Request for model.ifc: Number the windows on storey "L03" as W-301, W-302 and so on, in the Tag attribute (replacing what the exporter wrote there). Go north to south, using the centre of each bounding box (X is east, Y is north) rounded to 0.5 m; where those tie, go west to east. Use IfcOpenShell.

First a look at what the model holds.

```python
import ifcopenshell
import ifcopenshell.util.element
import ifcopenshell.util.placement

model = ifcopenshell.open("model.ifc")
print(model.schema)
storey = next(s for s in model.by_type("IfcBuildingStorey") if s.Name == "L03")
windows = [e for e in ifcopenshell.util.element.get_decomposition(storey) if e.is_a("IfcWindow")]
for e in sorted(windows, key=lambda e: e.id()):
    origin = ifcopenshell.util.placement.get_local_placement(e.ObjectPlacement)[:3, 3]
    print(e.id(), e.Tag, e.Name, origin.round(2) + 0.0, sep=" | ")
```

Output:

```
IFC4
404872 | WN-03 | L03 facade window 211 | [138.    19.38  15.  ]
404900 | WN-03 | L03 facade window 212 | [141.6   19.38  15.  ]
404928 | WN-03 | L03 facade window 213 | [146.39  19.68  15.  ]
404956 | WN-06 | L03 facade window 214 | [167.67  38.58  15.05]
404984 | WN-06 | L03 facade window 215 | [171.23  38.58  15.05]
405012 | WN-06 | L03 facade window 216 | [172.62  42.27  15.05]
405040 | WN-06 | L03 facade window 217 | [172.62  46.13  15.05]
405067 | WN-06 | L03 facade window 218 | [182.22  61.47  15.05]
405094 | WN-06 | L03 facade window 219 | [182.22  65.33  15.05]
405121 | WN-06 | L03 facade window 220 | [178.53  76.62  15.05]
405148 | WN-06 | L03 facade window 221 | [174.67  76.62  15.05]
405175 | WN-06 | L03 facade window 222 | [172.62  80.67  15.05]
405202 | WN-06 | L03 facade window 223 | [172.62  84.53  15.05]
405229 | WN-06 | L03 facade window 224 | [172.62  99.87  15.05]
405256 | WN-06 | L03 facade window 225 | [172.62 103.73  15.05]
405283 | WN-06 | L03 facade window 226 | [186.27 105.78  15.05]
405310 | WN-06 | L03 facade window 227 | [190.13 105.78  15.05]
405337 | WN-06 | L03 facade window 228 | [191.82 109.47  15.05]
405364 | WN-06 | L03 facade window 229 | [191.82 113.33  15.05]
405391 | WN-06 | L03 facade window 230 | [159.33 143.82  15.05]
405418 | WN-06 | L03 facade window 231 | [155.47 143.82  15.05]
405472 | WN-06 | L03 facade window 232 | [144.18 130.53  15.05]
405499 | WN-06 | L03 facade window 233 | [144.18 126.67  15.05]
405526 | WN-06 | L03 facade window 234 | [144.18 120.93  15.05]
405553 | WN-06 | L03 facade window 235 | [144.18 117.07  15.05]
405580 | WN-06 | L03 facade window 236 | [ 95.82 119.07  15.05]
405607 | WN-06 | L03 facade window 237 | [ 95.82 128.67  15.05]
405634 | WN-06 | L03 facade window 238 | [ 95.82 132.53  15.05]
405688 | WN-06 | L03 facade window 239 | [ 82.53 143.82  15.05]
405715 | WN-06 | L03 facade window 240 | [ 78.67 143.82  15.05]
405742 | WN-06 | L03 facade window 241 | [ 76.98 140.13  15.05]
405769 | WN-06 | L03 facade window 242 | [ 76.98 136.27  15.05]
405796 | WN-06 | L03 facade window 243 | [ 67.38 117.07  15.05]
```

```python
import ifcopenshell
import ifcopenshell.geom
import ifcopenshell.util.element
import ifcopenshell.util.shape

model = ifcopenshell.open("model.ifc")
settings = ifcopenshell.geom.settings()
settings.set("use-world-coords", True)


def centre(element):
    shape = ifcopenshell.geom.create_shape(settings, element)
    return ifcopenshell.util.shape.get_bbox_centroid(shape.geometry)


storey = next(s for s in model.by_type("IfcBuildingStorey") if s.Name == "L03")
windows = [e for e in ifcopenshell.util.element.get_decomposition(storey) if e.is_a("IfcWindow")]

# Insertion points can sit at a corner or the storey origin, so sort by the geometry (in metres).
centres = {e: centre(e) for e in windows}
windows.sort(key=lambda e: (-round(centres[e][1] / 0.5), centres[e][0]))

for i, e in enumerate(windows, start=1):
    number = f"W-3{i:02d}"
    e.Tag = number
    print(e.id(), number)

model.write("model_edited.ifc")
```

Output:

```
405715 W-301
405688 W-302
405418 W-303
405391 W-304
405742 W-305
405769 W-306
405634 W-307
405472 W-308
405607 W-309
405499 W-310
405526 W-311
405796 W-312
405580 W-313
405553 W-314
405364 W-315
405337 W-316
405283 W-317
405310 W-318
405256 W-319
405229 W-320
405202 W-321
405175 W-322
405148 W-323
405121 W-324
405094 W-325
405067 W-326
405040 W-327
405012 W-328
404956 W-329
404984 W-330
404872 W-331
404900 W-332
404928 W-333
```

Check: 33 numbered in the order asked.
